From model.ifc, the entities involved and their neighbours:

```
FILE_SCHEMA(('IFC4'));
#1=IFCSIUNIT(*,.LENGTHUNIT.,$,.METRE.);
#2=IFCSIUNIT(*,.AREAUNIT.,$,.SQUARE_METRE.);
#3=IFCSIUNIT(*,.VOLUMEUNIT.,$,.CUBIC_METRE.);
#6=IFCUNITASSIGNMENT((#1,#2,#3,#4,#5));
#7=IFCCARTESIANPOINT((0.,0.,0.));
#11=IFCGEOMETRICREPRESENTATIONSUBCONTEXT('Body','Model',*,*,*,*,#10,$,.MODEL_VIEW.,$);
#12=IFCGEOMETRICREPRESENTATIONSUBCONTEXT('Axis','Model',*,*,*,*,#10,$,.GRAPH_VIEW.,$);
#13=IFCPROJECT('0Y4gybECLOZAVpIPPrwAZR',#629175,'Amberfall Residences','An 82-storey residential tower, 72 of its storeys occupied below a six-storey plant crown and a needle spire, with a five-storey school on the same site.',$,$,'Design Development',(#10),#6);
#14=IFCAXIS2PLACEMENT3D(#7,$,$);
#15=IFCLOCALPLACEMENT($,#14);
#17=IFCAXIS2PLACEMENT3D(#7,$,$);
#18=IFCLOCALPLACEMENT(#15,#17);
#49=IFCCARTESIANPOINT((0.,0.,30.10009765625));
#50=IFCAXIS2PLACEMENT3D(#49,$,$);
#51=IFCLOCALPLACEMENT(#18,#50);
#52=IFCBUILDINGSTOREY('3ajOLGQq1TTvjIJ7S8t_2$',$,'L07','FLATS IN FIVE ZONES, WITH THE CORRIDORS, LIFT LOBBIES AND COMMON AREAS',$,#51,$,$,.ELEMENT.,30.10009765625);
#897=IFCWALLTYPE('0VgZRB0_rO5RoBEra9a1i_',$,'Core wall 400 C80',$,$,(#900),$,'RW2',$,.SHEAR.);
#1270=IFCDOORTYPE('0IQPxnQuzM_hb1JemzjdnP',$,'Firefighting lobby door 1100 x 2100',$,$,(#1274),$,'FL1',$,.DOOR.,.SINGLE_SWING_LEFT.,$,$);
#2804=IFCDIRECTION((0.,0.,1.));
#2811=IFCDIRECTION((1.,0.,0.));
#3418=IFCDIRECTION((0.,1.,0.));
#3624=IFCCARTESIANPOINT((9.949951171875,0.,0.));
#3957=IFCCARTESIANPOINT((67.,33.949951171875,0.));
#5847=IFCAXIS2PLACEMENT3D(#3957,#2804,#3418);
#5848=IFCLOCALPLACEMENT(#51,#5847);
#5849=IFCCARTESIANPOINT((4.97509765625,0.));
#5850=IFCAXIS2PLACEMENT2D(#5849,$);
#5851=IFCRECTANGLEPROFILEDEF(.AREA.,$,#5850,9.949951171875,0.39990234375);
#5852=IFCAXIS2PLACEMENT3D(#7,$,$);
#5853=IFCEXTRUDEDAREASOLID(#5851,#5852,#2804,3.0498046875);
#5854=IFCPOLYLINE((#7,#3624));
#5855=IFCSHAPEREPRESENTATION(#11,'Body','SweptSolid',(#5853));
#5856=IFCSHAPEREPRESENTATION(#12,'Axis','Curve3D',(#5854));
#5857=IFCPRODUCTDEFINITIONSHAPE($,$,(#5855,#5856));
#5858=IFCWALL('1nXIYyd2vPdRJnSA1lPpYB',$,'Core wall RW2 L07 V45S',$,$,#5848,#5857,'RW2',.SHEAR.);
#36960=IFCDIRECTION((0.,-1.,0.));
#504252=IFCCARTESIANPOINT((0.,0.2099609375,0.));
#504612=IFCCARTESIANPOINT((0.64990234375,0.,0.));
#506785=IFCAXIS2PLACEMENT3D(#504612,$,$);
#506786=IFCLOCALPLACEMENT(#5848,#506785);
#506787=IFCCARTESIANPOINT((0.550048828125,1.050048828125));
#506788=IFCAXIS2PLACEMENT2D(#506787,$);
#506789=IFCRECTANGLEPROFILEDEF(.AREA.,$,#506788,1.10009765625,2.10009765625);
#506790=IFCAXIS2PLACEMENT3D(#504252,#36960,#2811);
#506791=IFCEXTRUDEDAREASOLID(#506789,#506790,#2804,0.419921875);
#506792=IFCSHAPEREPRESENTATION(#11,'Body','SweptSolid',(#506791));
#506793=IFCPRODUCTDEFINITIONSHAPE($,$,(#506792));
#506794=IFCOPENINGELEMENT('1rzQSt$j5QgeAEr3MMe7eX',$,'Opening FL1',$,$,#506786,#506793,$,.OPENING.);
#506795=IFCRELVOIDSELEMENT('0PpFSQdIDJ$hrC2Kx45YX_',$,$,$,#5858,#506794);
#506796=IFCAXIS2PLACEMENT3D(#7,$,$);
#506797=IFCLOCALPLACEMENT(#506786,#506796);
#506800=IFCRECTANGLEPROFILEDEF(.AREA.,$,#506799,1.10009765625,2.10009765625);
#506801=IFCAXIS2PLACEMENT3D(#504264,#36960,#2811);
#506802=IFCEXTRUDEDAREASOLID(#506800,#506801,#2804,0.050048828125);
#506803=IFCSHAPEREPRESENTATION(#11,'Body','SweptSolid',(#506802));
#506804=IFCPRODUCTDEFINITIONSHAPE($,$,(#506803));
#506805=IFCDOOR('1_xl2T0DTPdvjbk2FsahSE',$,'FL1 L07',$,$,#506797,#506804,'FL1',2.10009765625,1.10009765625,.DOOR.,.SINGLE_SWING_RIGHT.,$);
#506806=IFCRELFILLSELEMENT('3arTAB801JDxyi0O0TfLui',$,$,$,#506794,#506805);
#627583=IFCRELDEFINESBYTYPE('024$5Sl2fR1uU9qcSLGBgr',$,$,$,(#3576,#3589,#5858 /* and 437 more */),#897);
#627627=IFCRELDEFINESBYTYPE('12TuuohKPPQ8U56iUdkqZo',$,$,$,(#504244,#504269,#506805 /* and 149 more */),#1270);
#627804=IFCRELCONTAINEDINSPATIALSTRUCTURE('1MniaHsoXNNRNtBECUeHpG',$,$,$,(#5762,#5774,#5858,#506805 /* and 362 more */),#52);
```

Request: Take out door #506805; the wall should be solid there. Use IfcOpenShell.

```python
import ifcopenshell
import ifcopenshell.api.feature
import ifcopenshell.api.root
import ifcopenshell.geom
import ifcopenshell.util.shape

model = ifcopenshell.open("model.ifc")
settings = ifcopenshell.geom.settings()


def volume(element):
    """Net volume in cubic metres, openings subtracted."""
    shape = ifcopenshell.geom.create_shape(settings, element)
    return ifcopenshell.util.shape.get_volume(shape.geometry)


door = model.by_id(506805)
opening = door.FillsVoids[0].RelatingOpeningElement
wall = opening.VoidsElements[0].RelatingBuildingElement
before = volume(wall)

ifcopenshell.api.root.remove_product(model, product=door)
ifcopenshell.api.feature.remove_feature(model, feature=opening)

after = volume(wall)

print(f"wall volume {before:.3f} -> {after:.3f} m3")

model.write("model-out.ifc")
```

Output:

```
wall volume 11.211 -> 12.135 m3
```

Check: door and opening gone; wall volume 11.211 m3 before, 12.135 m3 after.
